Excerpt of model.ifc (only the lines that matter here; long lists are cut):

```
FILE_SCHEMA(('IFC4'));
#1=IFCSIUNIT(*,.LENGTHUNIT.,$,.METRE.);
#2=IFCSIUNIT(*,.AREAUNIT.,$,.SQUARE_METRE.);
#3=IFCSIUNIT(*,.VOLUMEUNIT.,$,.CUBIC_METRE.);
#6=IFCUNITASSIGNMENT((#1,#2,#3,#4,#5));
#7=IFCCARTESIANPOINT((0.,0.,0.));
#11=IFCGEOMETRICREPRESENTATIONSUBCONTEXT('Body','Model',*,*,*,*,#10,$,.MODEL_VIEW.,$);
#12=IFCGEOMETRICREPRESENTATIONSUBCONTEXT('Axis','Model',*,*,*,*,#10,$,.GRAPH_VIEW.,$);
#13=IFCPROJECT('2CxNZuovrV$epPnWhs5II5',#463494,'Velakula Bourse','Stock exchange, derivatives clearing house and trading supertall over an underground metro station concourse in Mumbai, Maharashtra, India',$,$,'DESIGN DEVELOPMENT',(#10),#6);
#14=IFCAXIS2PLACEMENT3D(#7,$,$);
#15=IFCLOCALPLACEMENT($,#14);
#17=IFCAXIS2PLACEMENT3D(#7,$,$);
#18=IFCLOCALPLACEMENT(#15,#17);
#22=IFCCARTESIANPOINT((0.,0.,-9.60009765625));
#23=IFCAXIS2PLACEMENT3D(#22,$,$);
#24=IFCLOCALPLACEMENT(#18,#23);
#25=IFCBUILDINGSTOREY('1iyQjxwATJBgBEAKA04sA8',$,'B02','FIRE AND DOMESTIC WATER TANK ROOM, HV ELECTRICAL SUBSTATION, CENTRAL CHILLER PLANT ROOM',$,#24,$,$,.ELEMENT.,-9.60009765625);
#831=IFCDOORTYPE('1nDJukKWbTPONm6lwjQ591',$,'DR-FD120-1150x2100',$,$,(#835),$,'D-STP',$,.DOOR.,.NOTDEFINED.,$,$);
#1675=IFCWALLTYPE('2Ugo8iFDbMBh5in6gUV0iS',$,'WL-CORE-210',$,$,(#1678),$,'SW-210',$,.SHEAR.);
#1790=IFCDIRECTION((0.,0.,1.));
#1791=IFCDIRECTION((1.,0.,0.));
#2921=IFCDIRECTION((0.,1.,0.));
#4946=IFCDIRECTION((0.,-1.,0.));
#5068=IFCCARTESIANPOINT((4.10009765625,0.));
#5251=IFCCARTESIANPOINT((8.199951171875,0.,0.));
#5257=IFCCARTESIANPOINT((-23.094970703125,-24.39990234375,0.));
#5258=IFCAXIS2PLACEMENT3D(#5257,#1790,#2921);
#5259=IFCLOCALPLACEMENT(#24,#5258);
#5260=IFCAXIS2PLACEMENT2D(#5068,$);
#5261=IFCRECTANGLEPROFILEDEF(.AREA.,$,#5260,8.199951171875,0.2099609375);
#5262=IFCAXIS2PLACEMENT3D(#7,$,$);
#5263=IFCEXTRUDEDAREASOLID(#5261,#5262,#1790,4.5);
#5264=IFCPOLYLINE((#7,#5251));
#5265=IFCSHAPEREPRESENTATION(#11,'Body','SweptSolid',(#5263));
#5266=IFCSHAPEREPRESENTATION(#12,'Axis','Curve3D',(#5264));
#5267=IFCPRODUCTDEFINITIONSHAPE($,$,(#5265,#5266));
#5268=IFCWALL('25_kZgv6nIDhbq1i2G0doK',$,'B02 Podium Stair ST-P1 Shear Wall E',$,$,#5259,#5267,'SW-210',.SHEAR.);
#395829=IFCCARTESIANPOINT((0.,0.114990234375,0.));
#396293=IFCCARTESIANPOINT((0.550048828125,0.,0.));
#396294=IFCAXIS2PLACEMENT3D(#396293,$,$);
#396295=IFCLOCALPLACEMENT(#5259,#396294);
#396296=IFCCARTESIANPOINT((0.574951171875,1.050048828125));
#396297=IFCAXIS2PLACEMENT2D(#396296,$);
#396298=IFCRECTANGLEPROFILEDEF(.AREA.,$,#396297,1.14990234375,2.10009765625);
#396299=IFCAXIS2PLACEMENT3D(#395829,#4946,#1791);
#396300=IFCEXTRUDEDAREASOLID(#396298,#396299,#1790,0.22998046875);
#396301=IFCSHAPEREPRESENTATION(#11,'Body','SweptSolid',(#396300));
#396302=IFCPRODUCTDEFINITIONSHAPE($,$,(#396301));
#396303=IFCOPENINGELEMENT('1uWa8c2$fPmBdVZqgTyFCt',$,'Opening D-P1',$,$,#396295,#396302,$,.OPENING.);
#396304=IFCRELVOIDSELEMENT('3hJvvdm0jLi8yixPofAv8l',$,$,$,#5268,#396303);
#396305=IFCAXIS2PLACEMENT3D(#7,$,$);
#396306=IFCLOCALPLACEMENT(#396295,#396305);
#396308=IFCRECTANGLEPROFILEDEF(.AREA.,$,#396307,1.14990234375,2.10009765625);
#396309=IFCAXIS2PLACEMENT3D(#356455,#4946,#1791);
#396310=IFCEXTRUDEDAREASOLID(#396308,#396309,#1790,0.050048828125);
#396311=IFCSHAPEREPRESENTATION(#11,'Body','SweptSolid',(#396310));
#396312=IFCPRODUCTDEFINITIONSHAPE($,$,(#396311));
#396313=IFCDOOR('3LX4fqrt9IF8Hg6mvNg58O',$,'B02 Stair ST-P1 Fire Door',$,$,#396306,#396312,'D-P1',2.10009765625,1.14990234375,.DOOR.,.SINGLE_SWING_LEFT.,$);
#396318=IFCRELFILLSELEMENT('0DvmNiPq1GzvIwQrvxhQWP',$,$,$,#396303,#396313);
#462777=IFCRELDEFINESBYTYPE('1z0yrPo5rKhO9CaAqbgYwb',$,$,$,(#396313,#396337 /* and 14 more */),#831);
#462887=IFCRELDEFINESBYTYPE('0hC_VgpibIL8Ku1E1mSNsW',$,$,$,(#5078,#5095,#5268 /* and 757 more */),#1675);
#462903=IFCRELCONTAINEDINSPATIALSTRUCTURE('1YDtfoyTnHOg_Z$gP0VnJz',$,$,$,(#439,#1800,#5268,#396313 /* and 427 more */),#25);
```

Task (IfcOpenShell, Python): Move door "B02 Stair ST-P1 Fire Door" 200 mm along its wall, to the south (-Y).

```python
import ifcopenshell
import ifcopenshell.api.geometry
import ifcopenshell.util.placement

model = ifcopenshell.open("model.ifc")

door = model.by_id(396313)
opening = door.FillsVoids[0].RelatingOpeningElement
wall = opening.VoidsElements[0].RelatingBuildingElement

wall_matrix = ifcopenshell.util.placement.get_local_placement(wall.ObjectPlacement)
shift = wall_matrix[:3, 0] * -0.2
before = ifcopenshell.util.placement.get_local_placement(door.ObjectPlacement)[:3, 3].copy()

# The door is placed relative to its opening, so it follows when the opening moves.
matrix = ifcopenshell.util.placement.get_local_placement(opening.ObjectPlacement)
matrix[:3, 3] += shift
ifcopenshell.api.geometry.edit_object_placement(
    model, product=opening, matrix=matrix, is_si=False, should_transform_children=True
)

after = ifcopenshell.util.placement.get_local_placement(door.ObjectPlacement)[:3, 3]
print("door moved by", (after - before).round(3) + 0.0)

model.write("model_updated.ifc")
```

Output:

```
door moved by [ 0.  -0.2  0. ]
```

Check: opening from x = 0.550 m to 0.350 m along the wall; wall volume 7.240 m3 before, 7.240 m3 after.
